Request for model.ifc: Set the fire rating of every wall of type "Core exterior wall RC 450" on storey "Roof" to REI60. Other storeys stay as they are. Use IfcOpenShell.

First a look at what the model holds.

```python
import ifcopenshell
import ifcopenshell.util.element

model = ifcopenshell.open("model.ifc")
print(model.schema)
storey = next(s for s in model.by_type("IfcBuildingStorey") if s.Name == "Roof")
walls = [e for e in ifcopenshell.util.element.get_decomposition(storey) if e.is_a("IfcWall")]
seen = {}
for e in walls:
    element_type = ifcopenshell.util.element.get_type(e)
    key = (element_type.Name if element_type != e and element_type else None, ifcopenshell.util.element.get_pset(e, "Pset_WallCommon", "FireRating"))
    seen[key] = seen.get(key, 0) + 1
for (name, value), count in sorted(seen.items(), key=str):
    print(count, "x", name, "|", value)
```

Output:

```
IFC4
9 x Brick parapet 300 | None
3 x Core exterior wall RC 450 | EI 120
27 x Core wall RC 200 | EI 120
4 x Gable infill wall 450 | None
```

```python
import ifcopenshell
import ifcopenshell.api.pset
import ifcopenshell.util.element

model = ifcopenshell.open("model.ifc")

storey = next(s for s in model.by_type("IfcBuildingStorey") if s.Name == "Roof")
walls = [e for e in ifcopenshell.util.element.get_decomposition(storey) if e.is_a("IfcWall")]

count = 0
for e in walls:
    element_type = ifcopenshell.util.element.get_type(e)
    if element_type in (None, e) or element_type.Name != "Core exterior wall RC 450":
        continue
    # add_pset returns the element's existing set when there is one.
    pset = ifcopenshell.api.pset.add_pset(model, product=e, name="Pset_WallCommon")
    ifcopenshell.api.pset.edit_pset(model, pset=pset, properties={"FireRating": "REI60"})
    count += 1

print(count, "walls updated")

model.write("model-out.ifc")
```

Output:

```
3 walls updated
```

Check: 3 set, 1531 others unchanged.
